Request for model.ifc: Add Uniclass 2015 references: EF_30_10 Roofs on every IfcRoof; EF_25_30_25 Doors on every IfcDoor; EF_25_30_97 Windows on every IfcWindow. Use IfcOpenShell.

First a look at what the model holds.

```python
import ifcopenshell

model = ifcopenshell.open("model.ifc")
print(model.schema)
print("classifications:", [c.Name for c in model.by_type("IfcClassification")])
for ifc_class in ("IfcDoor", "IfcRoof", "IfcStair", "IfcWall", "IfcWindow"):
    print(ifc_class, len(model.by_type(ifc_class)))
```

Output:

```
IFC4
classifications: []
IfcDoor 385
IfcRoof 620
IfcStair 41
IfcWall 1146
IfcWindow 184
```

```python
import ifcopenshell
import ifcopenshell.api.classification

model = ifcopenshell.open("model.ifc")

system = ifcopenshell.api.classification.add_classification(model, classification="Uniclass 2015")

codes = {
    "IfcRoof": ("EF_30_10", "Roofs"),
    "IfcDoor": ("EF_25_30_25", "Doors"),
    "IfcWindow": ("EF_25_30_97", "Windows"),
}
for ifc_class, (code, name) in codes.items():
    products = model.by_type(ifc_class)
    ifcopenshell.api.classification.add_reference(
        model, products=products, classification=system, identification=code, name=name
    )
    print(code, len(products))

model.write("model-out.ifc")
```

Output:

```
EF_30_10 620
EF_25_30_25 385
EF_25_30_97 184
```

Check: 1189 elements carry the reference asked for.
